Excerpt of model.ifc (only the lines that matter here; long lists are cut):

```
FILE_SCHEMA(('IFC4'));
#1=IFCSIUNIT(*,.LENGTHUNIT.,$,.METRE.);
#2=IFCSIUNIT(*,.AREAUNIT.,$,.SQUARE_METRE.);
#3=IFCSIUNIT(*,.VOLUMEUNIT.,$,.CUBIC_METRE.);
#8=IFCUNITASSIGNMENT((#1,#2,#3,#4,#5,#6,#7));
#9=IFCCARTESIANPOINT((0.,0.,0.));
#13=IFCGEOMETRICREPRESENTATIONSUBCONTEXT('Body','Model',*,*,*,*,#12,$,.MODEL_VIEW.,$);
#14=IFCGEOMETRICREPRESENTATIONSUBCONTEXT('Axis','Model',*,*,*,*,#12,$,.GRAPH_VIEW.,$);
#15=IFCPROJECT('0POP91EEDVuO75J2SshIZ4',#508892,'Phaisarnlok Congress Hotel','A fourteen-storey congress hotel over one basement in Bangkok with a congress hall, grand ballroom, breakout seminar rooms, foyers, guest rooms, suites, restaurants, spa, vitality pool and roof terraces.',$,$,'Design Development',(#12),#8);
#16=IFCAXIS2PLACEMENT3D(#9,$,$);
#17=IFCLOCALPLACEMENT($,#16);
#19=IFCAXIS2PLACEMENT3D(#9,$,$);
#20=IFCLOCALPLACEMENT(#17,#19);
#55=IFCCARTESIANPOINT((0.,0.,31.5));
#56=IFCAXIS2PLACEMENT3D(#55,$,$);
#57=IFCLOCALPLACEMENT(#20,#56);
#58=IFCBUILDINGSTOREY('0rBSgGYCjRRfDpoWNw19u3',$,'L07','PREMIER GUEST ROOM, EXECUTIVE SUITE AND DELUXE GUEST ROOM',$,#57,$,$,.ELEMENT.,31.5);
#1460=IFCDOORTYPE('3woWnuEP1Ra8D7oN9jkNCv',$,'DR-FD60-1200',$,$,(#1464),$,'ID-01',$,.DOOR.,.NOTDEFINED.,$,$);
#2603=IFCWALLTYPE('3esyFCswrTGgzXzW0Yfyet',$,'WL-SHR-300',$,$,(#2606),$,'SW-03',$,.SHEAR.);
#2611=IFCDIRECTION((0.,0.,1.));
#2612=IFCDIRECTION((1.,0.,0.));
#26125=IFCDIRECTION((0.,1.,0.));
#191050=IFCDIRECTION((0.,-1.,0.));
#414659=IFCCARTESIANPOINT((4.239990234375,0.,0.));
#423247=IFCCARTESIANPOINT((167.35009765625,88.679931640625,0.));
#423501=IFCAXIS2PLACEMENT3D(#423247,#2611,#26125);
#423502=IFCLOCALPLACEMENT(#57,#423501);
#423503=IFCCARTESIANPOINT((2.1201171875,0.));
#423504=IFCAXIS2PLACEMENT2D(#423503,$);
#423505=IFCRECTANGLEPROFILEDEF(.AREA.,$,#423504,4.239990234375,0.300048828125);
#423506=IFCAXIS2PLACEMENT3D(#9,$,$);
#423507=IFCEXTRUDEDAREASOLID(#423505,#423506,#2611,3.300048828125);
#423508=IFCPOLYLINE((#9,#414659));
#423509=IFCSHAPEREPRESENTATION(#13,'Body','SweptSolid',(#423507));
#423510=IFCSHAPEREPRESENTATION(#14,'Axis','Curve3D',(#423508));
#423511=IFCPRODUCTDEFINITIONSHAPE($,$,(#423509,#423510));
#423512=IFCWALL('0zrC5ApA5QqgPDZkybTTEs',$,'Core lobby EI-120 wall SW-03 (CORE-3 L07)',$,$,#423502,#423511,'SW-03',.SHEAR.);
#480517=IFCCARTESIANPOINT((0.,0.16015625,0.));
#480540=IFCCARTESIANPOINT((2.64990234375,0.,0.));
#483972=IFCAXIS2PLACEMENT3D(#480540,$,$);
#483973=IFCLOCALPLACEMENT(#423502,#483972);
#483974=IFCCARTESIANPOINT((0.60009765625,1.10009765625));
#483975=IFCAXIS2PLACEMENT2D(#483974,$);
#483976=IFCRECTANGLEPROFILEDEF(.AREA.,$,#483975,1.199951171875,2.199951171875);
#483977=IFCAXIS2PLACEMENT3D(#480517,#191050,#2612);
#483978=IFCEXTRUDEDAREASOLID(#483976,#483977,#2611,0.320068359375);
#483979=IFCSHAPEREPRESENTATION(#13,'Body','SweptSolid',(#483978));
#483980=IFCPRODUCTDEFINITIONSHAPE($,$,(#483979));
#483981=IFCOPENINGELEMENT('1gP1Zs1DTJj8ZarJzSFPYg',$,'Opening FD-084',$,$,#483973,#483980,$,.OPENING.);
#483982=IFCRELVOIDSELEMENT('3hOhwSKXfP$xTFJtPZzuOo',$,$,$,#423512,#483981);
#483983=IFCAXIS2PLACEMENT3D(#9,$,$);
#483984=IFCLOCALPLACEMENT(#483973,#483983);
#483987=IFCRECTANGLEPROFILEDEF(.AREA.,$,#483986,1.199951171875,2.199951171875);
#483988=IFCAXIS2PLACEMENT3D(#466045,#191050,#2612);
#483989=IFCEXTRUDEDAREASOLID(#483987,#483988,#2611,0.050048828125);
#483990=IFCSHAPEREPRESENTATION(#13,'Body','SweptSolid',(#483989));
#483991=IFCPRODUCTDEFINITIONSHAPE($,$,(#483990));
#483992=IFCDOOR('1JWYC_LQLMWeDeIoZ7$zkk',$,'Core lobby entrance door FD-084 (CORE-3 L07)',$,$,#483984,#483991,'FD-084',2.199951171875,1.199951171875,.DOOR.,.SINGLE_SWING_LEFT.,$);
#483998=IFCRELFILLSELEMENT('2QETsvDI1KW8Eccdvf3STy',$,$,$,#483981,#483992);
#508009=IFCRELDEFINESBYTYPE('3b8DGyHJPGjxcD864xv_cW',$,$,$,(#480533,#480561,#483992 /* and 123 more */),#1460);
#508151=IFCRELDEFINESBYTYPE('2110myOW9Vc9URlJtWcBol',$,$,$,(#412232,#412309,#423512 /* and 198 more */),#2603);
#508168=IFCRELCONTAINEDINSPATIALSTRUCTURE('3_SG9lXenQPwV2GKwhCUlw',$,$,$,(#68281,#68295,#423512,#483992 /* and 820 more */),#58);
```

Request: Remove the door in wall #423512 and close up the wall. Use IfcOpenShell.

```python
import ifcopenshell
import ifcopenshell.api.feature
import ifcopenshell.api.root
import ifcopenshell.geom
import ifcopenshell.util.shape

model = ifcopenshell.open("model.ifc")
settings = ifcopenshell.geom.settings()


def volume(element):
    """Net volume in cubic metres, openings subtracted."""
    shape = ifcopenshell.geom.create_shape(settings, element)
    return ifcopenshell.util.shape.get_volume(shape.geometry)


door = model.by_id(483992)
opening = door.FillsVoids[0].RelatingOpeningElement
wall = opening.VoidsElements[0].RelatingBuildingElement
before = volume(wall)

ifcopenshell.api.root.remove_product(model, product=door)
ifcopenshell.api.feature.remove_feature(model, feature=opening)

after = volume(wall)

print(f"wall volume {before:.3f} -> {after:.3f} m3")

model.write("model_edited.ifc")
```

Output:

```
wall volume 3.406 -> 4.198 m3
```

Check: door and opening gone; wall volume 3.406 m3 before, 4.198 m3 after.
